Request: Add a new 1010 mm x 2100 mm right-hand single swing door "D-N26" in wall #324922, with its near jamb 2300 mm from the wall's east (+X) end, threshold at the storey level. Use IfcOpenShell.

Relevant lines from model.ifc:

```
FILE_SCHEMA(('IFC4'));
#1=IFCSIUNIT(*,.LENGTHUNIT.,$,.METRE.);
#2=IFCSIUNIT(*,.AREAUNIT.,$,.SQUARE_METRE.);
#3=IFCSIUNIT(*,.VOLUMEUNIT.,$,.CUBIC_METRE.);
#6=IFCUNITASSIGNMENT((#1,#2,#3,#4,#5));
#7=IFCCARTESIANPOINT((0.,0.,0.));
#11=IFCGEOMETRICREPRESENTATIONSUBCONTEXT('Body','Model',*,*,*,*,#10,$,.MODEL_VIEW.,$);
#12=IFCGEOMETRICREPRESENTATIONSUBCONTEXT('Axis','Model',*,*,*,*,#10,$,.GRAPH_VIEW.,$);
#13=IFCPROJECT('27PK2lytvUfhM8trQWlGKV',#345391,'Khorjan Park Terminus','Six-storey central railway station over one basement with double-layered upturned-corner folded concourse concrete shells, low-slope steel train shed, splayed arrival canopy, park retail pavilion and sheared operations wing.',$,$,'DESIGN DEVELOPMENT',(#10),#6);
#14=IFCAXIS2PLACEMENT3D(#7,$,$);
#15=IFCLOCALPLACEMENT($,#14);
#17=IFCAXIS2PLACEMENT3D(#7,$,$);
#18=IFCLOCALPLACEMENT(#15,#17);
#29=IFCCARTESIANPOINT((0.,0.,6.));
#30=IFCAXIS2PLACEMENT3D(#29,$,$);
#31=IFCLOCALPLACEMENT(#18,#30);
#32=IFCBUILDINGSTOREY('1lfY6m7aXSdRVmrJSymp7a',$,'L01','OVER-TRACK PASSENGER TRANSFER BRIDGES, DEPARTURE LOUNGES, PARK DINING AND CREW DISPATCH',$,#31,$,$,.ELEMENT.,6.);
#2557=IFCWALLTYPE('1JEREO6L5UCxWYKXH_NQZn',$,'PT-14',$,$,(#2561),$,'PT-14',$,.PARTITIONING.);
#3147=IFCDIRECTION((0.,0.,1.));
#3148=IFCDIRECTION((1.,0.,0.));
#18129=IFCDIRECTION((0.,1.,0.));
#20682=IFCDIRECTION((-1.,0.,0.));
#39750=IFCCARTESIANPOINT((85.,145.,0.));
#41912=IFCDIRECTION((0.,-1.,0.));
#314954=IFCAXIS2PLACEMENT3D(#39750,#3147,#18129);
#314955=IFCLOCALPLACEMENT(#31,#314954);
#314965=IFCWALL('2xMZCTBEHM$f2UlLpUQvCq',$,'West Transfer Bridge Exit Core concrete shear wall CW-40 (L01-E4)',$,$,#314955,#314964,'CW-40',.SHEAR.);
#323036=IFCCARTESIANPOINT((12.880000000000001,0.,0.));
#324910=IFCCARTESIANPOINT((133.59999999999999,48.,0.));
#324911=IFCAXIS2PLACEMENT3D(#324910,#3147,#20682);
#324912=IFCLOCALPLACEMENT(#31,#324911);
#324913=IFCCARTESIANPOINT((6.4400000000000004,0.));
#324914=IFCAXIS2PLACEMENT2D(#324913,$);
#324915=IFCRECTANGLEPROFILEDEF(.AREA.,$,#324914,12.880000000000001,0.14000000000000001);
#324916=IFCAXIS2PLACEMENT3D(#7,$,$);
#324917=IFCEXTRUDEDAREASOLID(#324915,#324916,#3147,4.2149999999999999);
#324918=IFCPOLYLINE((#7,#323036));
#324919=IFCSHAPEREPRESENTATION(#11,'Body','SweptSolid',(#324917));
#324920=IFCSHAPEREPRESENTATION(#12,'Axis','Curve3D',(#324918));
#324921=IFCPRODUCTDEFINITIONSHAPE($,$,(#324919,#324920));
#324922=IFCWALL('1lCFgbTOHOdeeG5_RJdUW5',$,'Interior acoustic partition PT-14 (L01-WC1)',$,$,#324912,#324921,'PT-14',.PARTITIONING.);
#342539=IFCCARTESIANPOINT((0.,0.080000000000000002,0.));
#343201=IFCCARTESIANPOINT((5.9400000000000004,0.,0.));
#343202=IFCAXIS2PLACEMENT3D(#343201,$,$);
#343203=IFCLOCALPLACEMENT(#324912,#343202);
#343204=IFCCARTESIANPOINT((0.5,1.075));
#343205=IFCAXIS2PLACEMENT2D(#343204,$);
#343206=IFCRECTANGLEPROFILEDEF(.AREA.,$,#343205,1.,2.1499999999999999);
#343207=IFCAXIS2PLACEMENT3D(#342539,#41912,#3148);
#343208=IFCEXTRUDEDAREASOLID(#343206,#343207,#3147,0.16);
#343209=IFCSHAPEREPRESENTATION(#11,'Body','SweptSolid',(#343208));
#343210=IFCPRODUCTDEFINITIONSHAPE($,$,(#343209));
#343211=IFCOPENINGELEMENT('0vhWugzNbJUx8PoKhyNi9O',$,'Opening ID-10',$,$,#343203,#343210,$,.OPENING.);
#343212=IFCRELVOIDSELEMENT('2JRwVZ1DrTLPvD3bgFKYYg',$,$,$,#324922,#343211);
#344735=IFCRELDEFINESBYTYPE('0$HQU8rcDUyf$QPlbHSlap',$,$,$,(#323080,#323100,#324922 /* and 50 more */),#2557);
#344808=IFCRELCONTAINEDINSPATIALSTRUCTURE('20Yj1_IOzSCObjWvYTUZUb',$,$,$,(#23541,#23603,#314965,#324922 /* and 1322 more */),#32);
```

```python
import numpy as np
import ifcopenshell
import ifcopenshell.api.feature
import ifcopenshell.api.geometry
import ifcopenshell.api.root
import ifcopenshell.api.spatial
import ifcopenshell.geom
import ifcopenshell.util.element
import ifcopenshell.util.placement
import ifcopenshell.util.representation
import ifcopenshell.util.shape
import ifcopenshell.util.unit

model = ifcopenshell.open("model.ifc")
unit_scale = ifcopenshell.util.unit.calculate_unit_scale(model)
settings = ifcopenshell.geom.settings()


def volume(element):
    """Net volume in cubic metres, openings subtracted."""
    shape = ifcopenshell.geom.create_shape(settings, element)
    return ifcopenshell.util.shape.get_volume(shape.geometry)


wall = model.by_guid("1lCFgbTOHOdeeG5_RJdUW5")
storey = ifcopenshell.util.element.get_container(wall, ifc_class="IfcBuildingStorey")
context = ifcopenshell.util.representation.get_context(model, "Model", "Body", "MODEL_VIEW")
before = volume(wall)

width, height, from_end, sill = 1.01, 2.1, 2.3, 0.0  # metres

# The wall runs along its own X axis, and the end named is its -X end.
wall_shape = ifcopenshell.geom.create_shape(settings, wall)
x, y, z = ifcopenshell.util.shape.get_vertices(wall_shape.geometry).T
start = x.min() + from_end
face, thickness = float(y.min()), float(y.max() - y.min())
wall_matrix = ifcopenshell.util.placement.get_local_placement(wall.ObjectPlacement)
level = ifcopenshell.util.placement.get_local_placement(storey.ObjectPlacement)[2, 3]


def in_wall(x, y):
    """Placement at x, y metres in the wall's axes, at sill height."""
    matrix = wall_matrix.copy()
    matrix[:, 3] = wall_matrix @ np.array([x / unit_scale, y / unit_scale, 0.0, 1.0])
    matrix[2, 3] = level + sill / unit_scale
    return matrix


# Opening: a box that overshoots both wall faces by 50 mm.
opening = ifcopenshell.api.root.create_entity(model, ifc_class="IfcOpeningElement", predefined_type="OPENING")
box = ifcopenshell.api.geometry.add_wall_representation(
    model, context=context, length=width, height=height, thickness=thickness + 0.1
)
ifcopenshell.api.geometry.assign_representation(model, product=opening, representation=box)
ifcopenshell.api.geometry.edit_object_placement(model, product=opening, matrix=in_wall(start, face - 0.05), is_si=False)
ifcopenshell.api.feature.add_feature(model, feature=opening, element=wall)

door = ifcopenshell.api.root.create_entity(model, ifc_class="IfcDoor", name="D-N26", predefined_type="DOOR")
door.OverallWidth, door.OverallHeight = width / unit_scale, height / unit_scale
door.OperationType = "SINGLE_SWING_RIGHT"
body = ifcopenshell.api.geometry.add_door_representation(
    model,
    context=context,
    overall_width=door.OverallWidth,
    overall_height=door.OverallHeight,
    operation_type="SINGLE_SWING_RIGHT",
    lining_properties={"LiningDepth": thickness / unit_scale, "ThresholdDepth": thickness / unit_scale},
)
ifcopenshell.api.geometry.assign_representation(model, product=door, representation=body)
ifcopenshell.api.spatial.assign_container(model, products=[door], relating_structure=storey)
ifcopenshell.api.feature.add_filling(model, opening=opening, element=door)

# The lining spans the wall, so the door starts at the wall face.
ifcopenshell.api.geometry.edit_object_placement(model, product=door, matrix=in_wall(start, face), is_si=False)

after = volume(wall)

print(f"wall volume {before:.3f} -> {after:.3f} m3")

model.write("model_updated.ifc")
```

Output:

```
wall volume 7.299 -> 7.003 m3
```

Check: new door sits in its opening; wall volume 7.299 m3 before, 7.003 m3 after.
